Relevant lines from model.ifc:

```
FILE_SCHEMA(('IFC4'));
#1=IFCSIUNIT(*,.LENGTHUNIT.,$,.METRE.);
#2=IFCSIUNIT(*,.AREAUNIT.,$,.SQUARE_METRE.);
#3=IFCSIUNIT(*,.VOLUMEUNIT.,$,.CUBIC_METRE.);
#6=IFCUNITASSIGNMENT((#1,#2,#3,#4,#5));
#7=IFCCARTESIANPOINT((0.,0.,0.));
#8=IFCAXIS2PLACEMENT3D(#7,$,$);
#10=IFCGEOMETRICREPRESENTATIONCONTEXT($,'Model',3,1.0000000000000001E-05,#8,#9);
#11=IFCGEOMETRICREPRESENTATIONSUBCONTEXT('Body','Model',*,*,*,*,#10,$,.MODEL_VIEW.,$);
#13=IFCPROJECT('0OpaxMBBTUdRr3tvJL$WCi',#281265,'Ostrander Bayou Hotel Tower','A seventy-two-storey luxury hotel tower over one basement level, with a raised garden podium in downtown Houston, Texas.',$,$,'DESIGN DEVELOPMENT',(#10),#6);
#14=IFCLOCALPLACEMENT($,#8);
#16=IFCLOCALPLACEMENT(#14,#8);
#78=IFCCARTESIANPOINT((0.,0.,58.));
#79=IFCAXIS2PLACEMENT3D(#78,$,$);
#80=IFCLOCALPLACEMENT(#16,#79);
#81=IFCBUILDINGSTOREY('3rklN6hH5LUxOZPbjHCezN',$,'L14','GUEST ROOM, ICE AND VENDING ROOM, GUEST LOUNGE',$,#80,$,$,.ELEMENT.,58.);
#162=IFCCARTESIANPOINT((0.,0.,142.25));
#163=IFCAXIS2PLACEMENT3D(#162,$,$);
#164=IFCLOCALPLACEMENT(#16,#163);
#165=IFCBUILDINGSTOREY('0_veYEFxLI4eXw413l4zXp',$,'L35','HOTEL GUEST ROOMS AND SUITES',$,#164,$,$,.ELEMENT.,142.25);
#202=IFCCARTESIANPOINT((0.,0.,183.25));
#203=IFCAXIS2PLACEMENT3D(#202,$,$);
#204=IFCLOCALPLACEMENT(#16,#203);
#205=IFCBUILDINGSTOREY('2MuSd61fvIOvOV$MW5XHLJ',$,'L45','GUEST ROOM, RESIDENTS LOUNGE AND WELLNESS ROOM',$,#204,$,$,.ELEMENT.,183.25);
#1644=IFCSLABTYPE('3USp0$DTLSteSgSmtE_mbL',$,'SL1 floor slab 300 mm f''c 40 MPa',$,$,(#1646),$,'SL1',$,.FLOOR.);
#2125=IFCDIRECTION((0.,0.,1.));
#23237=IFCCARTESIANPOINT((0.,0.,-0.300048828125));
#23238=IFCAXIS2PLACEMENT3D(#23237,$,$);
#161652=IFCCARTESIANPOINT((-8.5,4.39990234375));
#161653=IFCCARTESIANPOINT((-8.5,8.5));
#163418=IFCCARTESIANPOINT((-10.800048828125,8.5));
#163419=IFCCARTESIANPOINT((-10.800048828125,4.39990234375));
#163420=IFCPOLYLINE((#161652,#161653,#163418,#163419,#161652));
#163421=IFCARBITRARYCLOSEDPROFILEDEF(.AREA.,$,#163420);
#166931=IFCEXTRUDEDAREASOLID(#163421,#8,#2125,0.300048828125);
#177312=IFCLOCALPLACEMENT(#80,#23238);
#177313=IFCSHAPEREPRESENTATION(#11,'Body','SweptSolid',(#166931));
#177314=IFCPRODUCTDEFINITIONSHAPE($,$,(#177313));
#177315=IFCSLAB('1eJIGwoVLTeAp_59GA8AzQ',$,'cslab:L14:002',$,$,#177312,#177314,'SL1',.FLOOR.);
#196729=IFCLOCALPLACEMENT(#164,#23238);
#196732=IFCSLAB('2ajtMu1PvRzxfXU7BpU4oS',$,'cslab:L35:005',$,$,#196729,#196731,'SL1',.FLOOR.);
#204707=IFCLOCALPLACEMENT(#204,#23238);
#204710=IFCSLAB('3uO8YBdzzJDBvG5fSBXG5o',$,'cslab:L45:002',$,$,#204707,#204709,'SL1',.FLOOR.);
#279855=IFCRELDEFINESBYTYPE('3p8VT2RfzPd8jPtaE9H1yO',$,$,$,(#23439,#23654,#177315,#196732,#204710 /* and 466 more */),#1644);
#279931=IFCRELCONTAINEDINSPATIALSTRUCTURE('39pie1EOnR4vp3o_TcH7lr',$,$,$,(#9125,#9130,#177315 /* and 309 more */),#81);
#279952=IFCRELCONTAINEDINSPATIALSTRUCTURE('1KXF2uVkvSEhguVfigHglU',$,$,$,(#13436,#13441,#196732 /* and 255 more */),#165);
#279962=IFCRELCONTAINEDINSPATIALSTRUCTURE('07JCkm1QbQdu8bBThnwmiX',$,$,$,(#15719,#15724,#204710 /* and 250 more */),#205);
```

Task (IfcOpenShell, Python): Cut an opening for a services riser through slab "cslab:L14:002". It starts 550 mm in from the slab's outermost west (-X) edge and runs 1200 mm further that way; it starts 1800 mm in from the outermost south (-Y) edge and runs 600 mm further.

```python
import numpy as np
import ifcopenshell
import ifcopenshell.api.feature
import ifcopenshell.api.geometry
import ifcopenshell.api.root
import ifcopenshell.geom
import ifcopenshell.util.placement
import ifcopenshell.util.representation
import ifcopenshell.util.shape
import ifcopenshell.util.unit

model = ifcopenshell.open("model.ifc")
unit_scale = ifcopenshell.util.unit.calculate_unit_scale(model)
settings = ifcopenshell.geom.settings()


def volume(element):
    """Net volume in cubic metres, openings subtracted."""
    shape = ifcopenshell.geom.create_shape(settings, element)
    return ifcopenshell.util.shape.get_volume(shape.geometry)


slab = model.by_guid("1eJIGwoVLTeAp_59GA8AzQ")
before = volume(slab)

# Extent in the slab's own axes, in metres. The edges named are its -X and -Y sides.
slab_shape = ifcopenshell.geom.create_shape(settings, slab)
vertices = ifcopenshell.util.shape.get_vertices(slab_shape.geometry)
x_min, y_min, bottom = vertices.min(axis=0)
top = vertices[:, 2].max()

opening = ifcopenshell.api.root.create_entity(model, ifc_class="IfcOpeningElement", name="Services riser opening", predefined_type="OPENING")
context = ifcopenshell.util.representation.get_context(model, "Model", "Body", "MODEL_VIEW")
width, depth = 1.2, 0.6
outline = [(0.0, 0.0), (width, 0.0), (width, depth), (0.0, depth), (0.0, 0.0)]
# Overshoot both faces by 50 mm so the cut is clean.
shape = ifcopenshell.api.geometry.add_slab_representation(
    model, context=context, depth=top - bottom + 0.1, polyline=outline
)
ifcopenshell.api.geometry.assign_representation(model, product=opening, representation=shape)

matrix = ifcopenshell.util.placement.get_local_placement(slab.ObjectPlacement)
matrix[:, 3] = matrix @ np.append(np.array([x_min + 0.55, y_min + 1.8, bottom - 0.05]) / unit_scale, 1.0)
ifcopenshell.api.geometry.edit_object_placement(model, product=opening, matrix=matrix, is_si=False)
ifcopenshell.api.feature.add_feature(model, feature=opening, element=slab)

after = volume(slab)

print(f"slab volume {before:.3f} -> {after:.3f} m3")

model.write("model_updated.ifc")
```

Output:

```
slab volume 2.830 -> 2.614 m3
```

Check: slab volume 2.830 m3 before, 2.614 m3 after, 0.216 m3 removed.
